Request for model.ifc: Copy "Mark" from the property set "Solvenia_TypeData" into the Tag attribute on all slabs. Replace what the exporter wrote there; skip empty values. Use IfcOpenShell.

First a look at what the model holds.

```python
import ifcopenshell
import ifcopenshell.util.element

model = ifcopenshell.open("model.ifc")
print(model.schema)
slabs = model.by_type("IfcSlab")
print(len(slabs), "slabs")
for e in slabs[:8]:
    source = ifcopenshell.util.element.get_pset(e, "Solvenia_TypeData", "Mark")
    target = e.Tag
    print(e.id(), repr(source), repr(target), sep=" | ")
```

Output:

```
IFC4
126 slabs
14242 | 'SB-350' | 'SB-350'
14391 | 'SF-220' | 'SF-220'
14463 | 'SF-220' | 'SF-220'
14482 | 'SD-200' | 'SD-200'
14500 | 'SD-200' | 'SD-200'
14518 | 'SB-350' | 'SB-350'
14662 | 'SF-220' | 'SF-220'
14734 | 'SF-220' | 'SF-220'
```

```python
import ifcopenshell
import ifcopenshell.util.element

model = ifcopenshell.open("model.ifc")

count = 0
for e in model.by_type("IfcSlab"):
    value = ifcopenshell.util.element.get_pset(e, "Solvenia_TypeData", "Mark")
    current = e.Tag
    if not value or not value.strip() or current == value:
        continue
    e.Tag = value
    count += 1

print(count, "slabs updated")

model.write("model-out.ifc")
```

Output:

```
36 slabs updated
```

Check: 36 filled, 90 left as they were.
